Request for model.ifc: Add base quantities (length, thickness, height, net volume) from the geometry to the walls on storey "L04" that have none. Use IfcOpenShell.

First a look at what the model holds.

```python
import ifcopenshell
import ifcopenshell.util.element
import ifcopenshell.util.unit

model = ifcopenshell.open("model.ifc")
print(model.schema)
for unit_type in ("LENGTHUNIT", "AREAUNIT", "VOLUMEUNIT"):
    print(unit_type, ifcopenshell.util.unit.calculate_unit_scale(model, unit_type))
storey = next(s for s in model.by_type("IfcBuildingStorey") if s.Name == "L04")
walls = [e for e in ifcopenshell.util.element.get_decomposition(storey) if e.is_a("IfcWall")]
for e in sorted(walls, key=lambda e: e.id()):
    print(e.id(), e.is_a(), e.Name, list(ifcopenshell.util.element.get_psets(e, qtos_only=True)), sep=" | ")
```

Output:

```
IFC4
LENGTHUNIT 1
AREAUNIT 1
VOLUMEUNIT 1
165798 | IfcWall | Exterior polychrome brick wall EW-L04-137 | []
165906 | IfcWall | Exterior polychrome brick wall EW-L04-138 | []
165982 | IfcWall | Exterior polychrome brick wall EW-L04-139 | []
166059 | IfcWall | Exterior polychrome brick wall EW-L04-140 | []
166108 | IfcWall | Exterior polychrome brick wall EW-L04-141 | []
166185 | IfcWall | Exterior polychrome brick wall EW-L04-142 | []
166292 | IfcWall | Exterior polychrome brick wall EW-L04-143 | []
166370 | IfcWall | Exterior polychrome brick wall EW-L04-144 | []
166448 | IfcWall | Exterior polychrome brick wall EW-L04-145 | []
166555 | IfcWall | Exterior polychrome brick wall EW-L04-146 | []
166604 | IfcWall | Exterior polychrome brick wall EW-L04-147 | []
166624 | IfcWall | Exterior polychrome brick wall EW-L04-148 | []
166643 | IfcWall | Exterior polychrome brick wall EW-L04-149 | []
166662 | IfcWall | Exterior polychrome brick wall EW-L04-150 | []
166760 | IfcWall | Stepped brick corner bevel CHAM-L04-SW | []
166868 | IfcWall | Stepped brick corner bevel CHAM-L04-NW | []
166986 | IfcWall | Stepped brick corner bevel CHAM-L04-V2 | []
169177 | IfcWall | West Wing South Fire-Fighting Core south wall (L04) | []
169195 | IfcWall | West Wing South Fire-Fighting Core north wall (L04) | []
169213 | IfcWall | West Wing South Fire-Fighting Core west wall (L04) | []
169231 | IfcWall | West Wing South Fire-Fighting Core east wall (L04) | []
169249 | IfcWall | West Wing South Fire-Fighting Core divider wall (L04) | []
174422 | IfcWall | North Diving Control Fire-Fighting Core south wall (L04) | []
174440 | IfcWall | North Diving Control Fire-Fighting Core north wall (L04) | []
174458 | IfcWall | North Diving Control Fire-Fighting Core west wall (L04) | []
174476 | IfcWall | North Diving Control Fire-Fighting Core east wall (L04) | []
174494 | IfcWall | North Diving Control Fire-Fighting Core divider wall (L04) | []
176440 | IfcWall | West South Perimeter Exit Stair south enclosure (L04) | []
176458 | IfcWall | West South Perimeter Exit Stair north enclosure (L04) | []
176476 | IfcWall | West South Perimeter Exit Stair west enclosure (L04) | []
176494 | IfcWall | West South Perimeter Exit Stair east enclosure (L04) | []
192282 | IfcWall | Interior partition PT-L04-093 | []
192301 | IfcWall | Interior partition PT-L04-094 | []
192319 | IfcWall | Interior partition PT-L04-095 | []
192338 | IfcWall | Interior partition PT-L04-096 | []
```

```python
import ifcopenshell
import ifcopenshell.api.pset
import ifcopenshell.geom
import ifcopenshell.util.element
import ifcopenshell.util.shape
import ifcopenshell.util.unit

model = ifcopenshell.open("model.ifc")
unit_scale = ifcopenshell.util.unit.calculate_unit_scale(model)
volume_scale = ifcopenshell.util.unit.calculate_unit_scale(model, "VOLUMEUNIT")
settings = ifcopenshell.geom.settings()

storey = next(s for s in model.by_type("IfcBuildingStorey") if s.Name == "L04")
walls = [e for e in ifcopenshell.util.element.get_decomposition(storey) if e.is_a("IfcWall")]

for e in sorted(walls, key=lambda e: e.id()):
    if ifcopenshell.util.element.get_psets(e, qtos_only=True, should_inherit=False):
        continue
    # Geometry comes back in metres, in the element's own axes.
    shape = ifcopenshell.geom.create_shape(settings, e)
    values = {
        "Length": ifcopenshell.util.shape.get_x(shape.geometry) / unit_scale,
        "Width": ifcopenshell.util.shape.get_y(shape.geometry) / unit_scale,
        "Height": ifcopenshell.util.shape.get_z(shape.geometry) / unit_scale,
        "NetVolume": ifcopenshell.util.shape.get_volume(shape.geometry) / volume_scale,
    }
    qto = ifcopenshell.api.pset.add_qto(model, product=e, name="Qto_WallBaseQuantities")
    ifcopenshell.api.pset.edit_qto(model, qto=qto, properties=values)
    print(e.id(), {k: round(v, 3) for k, v in values.items()})

model.write("model_edited.ifc")
```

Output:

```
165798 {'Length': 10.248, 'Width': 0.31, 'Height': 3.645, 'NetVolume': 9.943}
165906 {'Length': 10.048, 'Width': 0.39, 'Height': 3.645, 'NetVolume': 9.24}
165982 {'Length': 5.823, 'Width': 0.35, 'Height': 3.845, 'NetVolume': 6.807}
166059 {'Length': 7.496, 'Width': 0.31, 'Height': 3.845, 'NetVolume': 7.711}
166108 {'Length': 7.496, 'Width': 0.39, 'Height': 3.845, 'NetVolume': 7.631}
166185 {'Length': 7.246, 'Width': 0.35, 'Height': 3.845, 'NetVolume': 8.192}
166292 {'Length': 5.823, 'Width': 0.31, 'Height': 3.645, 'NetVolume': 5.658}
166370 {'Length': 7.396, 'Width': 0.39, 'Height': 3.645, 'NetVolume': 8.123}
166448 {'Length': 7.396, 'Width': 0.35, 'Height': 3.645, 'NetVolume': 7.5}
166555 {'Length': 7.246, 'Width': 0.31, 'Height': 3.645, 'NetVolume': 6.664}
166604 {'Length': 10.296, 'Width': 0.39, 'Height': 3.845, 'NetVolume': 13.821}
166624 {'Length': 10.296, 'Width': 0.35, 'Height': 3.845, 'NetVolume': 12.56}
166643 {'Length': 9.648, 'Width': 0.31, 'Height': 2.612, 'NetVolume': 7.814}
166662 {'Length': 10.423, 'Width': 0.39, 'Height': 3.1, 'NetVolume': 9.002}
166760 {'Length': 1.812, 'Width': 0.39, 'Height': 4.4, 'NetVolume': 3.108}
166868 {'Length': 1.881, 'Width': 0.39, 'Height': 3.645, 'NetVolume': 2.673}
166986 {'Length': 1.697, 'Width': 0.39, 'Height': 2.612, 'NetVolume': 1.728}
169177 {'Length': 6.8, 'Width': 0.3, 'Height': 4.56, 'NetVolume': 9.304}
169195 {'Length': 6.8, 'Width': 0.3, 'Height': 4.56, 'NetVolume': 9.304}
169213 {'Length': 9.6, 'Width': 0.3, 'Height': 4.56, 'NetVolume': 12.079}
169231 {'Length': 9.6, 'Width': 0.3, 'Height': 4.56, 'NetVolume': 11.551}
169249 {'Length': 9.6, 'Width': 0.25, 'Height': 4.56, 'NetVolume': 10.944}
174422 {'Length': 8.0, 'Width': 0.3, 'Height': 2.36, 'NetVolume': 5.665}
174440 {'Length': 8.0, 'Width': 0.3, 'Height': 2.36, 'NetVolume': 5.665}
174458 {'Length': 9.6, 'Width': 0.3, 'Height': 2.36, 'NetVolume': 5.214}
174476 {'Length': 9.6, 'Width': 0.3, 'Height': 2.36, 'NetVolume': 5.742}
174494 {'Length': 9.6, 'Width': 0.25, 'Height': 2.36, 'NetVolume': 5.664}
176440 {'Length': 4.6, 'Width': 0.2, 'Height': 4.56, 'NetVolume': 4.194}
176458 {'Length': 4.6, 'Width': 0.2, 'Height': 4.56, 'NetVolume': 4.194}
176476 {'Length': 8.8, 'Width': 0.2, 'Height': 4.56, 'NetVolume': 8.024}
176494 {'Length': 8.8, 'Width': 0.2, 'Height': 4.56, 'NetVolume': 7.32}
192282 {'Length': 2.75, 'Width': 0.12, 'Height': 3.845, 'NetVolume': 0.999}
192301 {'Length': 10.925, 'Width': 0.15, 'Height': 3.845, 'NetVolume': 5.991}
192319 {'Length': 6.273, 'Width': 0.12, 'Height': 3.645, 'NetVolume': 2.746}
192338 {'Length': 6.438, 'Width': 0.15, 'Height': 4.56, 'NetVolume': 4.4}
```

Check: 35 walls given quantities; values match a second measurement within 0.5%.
